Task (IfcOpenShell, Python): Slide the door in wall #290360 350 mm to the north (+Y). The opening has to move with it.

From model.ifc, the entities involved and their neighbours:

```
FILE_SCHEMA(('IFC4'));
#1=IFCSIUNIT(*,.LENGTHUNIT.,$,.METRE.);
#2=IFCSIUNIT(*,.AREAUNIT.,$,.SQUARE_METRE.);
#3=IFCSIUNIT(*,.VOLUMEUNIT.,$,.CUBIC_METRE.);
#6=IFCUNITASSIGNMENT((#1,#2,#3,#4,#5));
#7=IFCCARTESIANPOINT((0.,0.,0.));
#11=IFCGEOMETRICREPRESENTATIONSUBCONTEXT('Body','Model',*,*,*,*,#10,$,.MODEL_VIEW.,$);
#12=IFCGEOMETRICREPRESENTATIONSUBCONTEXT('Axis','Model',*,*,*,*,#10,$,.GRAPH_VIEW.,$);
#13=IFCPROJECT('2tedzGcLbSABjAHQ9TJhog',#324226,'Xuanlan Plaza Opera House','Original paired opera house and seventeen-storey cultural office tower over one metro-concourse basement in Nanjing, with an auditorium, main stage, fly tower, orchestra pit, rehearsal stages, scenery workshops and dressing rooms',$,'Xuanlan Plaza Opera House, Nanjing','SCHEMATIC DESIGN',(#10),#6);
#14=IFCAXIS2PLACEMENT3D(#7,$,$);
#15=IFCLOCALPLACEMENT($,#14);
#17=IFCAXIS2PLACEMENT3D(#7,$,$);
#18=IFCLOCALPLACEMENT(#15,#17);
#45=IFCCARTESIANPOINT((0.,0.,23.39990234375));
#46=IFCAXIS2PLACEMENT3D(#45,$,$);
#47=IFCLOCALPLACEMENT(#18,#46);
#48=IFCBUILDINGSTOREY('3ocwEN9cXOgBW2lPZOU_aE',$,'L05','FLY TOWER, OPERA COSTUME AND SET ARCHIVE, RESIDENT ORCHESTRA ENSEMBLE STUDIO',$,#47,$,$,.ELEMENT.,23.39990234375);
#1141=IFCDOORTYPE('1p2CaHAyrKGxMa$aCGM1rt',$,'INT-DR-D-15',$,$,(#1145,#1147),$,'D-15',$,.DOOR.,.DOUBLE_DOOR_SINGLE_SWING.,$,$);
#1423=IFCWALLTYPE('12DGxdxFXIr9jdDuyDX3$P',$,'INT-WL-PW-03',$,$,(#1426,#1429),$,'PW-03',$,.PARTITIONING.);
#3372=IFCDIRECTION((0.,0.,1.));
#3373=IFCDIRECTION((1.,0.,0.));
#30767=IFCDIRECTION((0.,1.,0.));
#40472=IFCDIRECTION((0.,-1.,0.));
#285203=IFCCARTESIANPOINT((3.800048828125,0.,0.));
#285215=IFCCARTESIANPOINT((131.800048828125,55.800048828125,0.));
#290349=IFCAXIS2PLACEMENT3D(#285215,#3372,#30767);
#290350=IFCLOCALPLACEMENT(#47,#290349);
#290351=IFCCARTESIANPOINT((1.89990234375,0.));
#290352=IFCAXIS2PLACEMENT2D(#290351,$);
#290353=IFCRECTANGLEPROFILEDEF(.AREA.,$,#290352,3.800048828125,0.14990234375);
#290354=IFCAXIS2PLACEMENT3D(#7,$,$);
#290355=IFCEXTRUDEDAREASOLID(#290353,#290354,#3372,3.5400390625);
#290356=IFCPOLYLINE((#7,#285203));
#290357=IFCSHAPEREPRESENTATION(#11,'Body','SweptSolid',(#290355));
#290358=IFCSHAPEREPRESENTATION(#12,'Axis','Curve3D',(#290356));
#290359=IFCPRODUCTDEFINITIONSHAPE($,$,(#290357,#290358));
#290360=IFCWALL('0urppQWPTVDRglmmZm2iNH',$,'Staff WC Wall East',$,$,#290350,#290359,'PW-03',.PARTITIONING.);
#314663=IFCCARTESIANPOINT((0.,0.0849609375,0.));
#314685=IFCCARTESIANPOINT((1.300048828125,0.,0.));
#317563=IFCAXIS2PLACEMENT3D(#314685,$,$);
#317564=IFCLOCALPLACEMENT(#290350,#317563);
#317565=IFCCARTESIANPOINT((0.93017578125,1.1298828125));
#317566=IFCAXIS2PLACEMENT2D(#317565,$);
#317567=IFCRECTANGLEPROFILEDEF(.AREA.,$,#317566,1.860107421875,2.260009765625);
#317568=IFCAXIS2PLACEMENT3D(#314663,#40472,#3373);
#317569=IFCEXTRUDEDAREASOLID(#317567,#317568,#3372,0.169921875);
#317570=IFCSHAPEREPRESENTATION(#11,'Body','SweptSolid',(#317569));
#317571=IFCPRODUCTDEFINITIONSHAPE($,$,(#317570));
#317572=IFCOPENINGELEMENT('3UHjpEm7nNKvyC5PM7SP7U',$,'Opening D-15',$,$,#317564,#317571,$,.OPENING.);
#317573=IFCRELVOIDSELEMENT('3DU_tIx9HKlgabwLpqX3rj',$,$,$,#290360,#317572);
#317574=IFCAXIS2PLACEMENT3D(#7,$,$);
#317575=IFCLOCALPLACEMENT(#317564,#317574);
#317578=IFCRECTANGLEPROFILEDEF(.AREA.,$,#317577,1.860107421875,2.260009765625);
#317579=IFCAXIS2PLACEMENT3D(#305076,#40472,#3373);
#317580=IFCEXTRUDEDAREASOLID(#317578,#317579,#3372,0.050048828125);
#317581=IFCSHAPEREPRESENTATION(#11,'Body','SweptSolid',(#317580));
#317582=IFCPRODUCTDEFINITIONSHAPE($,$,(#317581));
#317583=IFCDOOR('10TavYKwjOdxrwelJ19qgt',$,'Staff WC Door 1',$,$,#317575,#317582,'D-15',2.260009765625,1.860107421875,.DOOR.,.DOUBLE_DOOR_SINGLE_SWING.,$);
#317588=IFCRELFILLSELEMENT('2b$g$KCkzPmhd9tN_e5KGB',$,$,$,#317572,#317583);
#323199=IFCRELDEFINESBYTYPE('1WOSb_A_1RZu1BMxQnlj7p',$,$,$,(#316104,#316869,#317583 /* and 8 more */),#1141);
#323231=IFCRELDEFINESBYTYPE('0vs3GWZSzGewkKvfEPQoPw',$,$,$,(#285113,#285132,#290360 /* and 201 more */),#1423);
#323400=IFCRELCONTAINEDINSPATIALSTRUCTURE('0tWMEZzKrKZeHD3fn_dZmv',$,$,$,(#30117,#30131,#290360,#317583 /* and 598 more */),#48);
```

```python
import ifcopenshell
import ifcopenshell.api.geometry
import ifcopenshell.util.placement
import ifcopenshell.util.unit

model = ifcopenshell.open("model.ifc")
unit_scale = ifcopenshell.util.unit.calculate_unit_scale(model)

door = model.by_id(317583)
opening = door.FillsVoids[0].RelatingOpeningElement
wall = opening.VoidsElements[0].RelatingBuildingElement

wall_matrix = ifcopenshell.util.placement.get_local_placement(wall.ObjectPlacement)
shift = wall_matrix[:3, 0] * 0.35 / unit_scale
before = ifcopenshell.util.placement.get_local_placement(door.ObjectPlacement)[:3, 3].copy()

# The door is placed relative to its opening, so it follows when the opening moves.
matrix = ifcopenshell.util.placement.get_local_placement(opening.ObjectPlacement)
matrix[:3, 3] += shift
ifcopenshell.api.geometry.edit_object_placement(
    model, product=opening, matrix=matrix, is_si=False, should_transform_children=True
)

after = ifcopenshell.util.placement.get_local_placement(door.ObjectPlacement)[:3, 3]
print("door moved by", (after - before).round(3) + 0.0)

model.write("model_v2.ifc")
```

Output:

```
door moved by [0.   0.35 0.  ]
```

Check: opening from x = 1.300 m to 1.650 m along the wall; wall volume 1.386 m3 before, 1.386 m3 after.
